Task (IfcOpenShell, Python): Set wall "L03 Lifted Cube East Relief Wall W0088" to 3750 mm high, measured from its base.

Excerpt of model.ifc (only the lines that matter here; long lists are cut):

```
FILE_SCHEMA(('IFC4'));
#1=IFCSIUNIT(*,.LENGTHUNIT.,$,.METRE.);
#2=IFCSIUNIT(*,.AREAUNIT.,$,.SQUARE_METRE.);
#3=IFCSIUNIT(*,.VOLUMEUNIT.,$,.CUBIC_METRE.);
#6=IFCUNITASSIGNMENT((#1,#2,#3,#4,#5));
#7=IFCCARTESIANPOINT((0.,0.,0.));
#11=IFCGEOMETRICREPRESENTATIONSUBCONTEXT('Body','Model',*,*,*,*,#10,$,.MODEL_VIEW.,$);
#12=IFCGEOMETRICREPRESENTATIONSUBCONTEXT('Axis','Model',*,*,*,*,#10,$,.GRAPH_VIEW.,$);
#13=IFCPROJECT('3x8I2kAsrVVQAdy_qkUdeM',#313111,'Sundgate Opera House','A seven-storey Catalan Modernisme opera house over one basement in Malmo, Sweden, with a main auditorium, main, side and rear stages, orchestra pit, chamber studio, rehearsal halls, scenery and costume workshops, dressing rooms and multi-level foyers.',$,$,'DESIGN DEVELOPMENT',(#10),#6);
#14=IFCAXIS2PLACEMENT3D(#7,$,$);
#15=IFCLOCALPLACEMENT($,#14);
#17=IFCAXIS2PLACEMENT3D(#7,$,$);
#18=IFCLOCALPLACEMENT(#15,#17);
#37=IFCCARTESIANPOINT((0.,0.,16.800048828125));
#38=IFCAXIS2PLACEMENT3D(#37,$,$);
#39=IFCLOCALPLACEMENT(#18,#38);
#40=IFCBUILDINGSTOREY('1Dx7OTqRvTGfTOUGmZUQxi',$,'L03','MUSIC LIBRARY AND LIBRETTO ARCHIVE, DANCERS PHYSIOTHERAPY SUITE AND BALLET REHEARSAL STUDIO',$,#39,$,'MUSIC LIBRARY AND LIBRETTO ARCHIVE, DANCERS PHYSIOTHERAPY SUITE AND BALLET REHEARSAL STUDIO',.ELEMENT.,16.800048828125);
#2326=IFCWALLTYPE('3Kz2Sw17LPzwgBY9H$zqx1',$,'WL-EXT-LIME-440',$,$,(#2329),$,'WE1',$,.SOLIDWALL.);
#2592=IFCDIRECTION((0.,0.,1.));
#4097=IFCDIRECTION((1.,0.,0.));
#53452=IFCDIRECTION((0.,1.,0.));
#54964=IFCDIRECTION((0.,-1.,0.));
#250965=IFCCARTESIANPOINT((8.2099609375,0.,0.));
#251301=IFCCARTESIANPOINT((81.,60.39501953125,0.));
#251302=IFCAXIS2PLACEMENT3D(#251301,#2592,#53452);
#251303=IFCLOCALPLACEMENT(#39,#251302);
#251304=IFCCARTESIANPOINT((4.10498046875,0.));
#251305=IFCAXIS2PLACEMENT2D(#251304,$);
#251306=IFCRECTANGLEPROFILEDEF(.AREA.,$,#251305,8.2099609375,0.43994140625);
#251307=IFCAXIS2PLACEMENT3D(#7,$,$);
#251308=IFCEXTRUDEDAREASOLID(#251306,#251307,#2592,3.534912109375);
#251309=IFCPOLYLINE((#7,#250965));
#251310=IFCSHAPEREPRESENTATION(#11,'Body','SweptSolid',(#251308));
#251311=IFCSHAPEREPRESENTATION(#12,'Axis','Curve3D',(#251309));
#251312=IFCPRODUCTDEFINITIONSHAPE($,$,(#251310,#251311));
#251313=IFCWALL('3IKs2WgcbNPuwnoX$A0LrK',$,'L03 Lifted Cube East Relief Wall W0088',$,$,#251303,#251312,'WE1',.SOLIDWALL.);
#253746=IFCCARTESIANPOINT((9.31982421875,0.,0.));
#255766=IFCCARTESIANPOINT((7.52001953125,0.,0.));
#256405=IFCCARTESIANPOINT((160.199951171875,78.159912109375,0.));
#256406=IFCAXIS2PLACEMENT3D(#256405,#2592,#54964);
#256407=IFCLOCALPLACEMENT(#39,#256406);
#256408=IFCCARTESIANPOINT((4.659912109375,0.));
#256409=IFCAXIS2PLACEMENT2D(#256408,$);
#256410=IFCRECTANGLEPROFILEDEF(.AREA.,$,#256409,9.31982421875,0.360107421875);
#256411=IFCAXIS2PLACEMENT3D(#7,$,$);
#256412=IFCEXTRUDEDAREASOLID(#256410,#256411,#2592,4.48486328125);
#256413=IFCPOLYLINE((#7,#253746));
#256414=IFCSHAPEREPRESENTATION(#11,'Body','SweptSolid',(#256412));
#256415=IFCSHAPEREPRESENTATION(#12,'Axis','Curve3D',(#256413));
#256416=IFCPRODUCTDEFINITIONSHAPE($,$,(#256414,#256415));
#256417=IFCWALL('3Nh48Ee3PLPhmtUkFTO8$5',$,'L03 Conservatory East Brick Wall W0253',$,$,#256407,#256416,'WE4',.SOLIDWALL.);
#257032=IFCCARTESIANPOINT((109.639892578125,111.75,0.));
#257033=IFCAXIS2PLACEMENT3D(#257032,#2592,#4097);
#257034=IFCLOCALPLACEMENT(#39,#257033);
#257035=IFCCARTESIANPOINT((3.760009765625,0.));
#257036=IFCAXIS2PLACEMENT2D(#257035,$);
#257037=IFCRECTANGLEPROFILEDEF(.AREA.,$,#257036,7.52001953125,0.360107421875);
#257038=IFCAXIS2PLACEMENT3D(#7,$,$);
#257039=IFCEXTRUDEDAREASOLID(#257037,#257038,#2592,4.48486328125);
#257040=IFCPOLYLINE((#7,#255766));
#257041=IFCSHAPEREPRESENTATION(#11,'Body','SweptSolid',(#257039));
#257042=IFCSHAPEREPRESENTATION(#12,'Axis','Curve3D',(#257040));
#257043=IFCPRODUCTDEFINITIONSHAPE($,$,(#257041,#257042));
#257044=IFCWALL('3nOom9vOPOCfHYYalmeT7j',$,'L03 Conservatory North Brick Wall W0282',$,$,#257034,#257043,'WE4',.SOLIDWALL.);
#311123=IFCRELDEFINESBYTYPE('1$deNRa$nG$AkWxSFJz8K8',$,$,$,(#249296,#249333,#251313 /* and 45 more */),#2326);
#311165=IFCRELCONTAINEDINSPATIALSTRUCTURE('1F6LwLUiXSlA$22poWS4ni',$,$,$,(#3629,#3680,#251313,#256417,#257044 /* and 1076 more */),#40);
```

```python
import ifcopenshell
import ifcopenshell.geom
import ifcopenshell.util.representation
import ifcopenshell.util.shape
import ifcopenshell.util.unit

model = ifcopenshell.open("model.ifc")
unit_scale = ifcopenshell.util.unit.calculate_unit_scale(model)
settings = ifcopenshell.geom.settings()


def volume(element):
    """Net volume in cubic metres, openings subtracted."""
    shape = ifcopenshell.geom.create_shape(settings, element)
    return ifcopenshell.util.shape.get_volume(shape.geometry)


wall = model.by_guid("3IKs2WgcbNPuwnoX$A0LrK")
before = volume(wall)

body = ifcopenshell.util.representation.get_representation(wall, "Model", "Body")
solid = body.Items[0]
old_height = solid.Depth
solid.Depth = 3.75 / unit_scale
after = volume(wall)

print(f"height {old_height:g} -> {solid.Depth:g}, volume {before:.3f} -> {after:.3f} m3")

model.write("model_updated.ifc")
```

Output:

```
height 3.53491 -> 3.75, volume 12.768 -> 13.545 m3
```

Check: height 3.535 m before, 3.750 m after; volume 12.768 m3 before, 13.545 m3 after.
